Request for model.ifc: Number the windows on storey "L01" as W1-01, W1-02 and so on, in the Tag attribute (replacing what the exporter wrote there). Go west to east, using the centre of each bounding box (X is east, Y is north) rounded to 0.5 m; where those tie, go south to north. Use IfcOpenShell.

First a look at what the model holds.

```python
import ifcopenshell
import ifcopenshell.util.element
import ifcopenshell.util.placement

model = ifcopenshell.open("model.ifc")
print(model.schema)
storey = next(s for s in model.by_type("IfcBuildingStorey") if s.Name == "L01")
windows = [e for e in ifcopenshell.util.element.get_decomposition(storey) if e.is_a("IfcWindow")]
for e in sorted(windows, key=lambda e: e.id()):
    origin = ifcopenshell.util.placement.get_local_placement(e.ObjectPlacement)[:3, 3]
    print(e.id(), e.Tag, e.Name, origin.round(2) + 0.0, sep=" | ")
```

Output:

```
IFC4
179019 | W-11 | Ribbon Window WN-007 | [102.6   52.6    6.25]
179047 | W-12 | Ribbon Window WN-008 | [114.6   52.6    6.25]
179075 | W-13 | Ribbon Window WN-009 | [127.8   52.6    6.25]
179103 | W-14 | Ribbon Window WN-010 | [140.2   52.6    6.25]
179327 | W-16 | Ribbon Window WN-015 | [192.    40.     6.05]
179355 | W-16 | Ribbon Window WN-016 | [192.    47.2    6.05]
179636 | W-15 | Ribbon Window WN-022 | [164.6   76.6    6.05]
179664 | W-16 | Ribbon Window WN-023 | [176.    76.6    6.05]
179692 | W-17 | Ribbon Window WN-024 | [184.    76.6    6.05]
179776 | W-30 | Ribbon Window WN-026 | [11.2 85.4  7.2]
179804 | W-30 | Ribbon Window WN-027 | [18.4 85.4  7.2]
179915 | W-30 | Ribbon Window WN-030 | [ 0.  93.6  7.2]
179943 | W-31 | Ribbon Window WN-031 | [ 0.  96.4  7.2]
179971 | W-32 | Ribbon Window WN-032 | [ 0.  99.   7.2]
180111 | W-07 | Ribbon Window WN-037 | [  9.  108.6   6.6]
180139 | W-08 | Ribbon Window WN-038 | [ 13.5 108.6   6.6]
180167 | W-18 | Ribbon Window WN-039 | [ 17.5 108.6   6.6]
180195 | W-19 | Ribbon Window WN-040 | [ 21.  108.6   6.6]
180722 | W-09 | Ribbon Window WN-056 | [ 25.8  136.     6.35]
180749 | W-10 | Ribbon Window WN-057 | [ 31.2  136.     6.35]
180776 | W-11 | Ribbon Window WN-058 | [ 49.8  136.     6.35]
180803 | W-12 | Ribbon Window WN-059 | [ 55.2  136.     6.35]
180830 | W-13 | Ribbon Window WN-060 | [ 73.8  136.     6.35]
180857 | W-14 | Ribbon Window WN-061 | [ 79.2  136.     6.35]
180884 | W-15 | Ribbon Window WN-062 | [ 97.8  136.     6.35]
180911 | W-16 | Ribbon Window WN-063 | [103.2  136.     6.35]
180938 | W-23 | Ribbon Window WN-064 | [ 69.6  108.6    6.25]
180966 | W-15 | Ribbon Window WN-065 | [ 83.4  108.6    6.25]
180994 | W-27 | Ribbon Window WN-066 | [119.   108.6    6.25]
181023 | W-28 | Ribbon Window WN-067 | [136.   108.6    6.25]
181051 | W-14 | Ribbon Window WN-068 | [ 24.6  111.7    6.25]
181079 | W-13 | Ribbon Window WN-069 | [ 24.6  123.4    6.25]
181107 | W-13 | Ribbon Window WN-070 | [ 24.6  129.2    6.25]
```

```python
import ifcopenshell
import ifcopenshell.geom
import ifcopenshell.util.element
import ifcopenshell.util.shape

model = ifcopenshell.open("model.ifc")
settings = ifcopenshell.geom.settings()
settings.set("use-world-coords", True)


def centre(element):
    shape = ifcopenshell.geom.create_shape(settings, element)
    return ifcopenshell.util.shape.get_bbox_centroid(shape.geometry)


storey = next(s for s in model.by_type("IfcBuildingStorey") if s.Name == "L01")
windows = [e for e in ifcopenshell.util.element.get_decomposition(storey) if e.is_a("IfcWindow")]

# Insertion points can sit at a corner or the storey origin, so sort by the geometry (in metres).
centres = {e: centre(e) for e in windows}
windows.sort(key=lambda e: (round(centres[e][0] / 0.5), centres[e][1]))

for i, e in enumerate(windows, start=1):
    number = f"W1-{i:02d}"
    e.Tag = number
    print(e.id(), number)

model.write("model-out.ifc")
```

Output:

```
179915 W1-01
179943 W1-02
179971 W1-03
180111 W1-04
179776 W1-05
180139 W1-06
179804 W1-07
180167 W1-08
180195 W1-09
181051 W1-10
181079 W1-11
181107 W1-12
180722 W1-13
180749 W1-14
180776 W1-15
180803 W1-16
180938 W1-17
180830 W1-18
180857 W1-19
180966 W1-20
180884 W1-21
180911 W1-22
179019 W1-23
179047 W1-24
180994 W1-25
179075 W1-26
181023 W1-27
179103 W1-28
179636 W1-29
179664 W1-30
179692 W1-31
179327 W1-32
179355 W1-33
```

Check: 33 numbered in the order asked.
